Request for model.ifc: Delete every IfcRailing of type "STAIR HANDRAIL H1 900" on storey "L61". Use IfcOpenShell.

First a look at what the model holds.

```python
import ifcopenshell
import ifcopenshell.util.element

model = ifcopenshell.open("model.ifc")
print(model.schema)
storey = next(s for s in model.by_type("IfcBuildingStorey") if s.Name == "L61")
railings = [e for e in ifcopenshell.util.element.get_decomposition(storey) if e.is_a("IfcRailing")]
seen = {}
for e in railings:
    element_type = ifcopenshell.util.element.get_type(e)
    name = element_type.Name if element_type not in (None, e) else None
    seen[name] = seen.get(name, 0) + 1
for name, count in sorted(seen.items(), key=str):
    print(count, "x", name)
```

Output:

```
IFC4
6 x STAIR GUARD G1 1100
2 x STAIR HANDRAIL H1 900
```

```python
import ifcopenshell
import ifcopenshell.api.root
import ifcopenshell.util.element

model = ifcopenshell.open("model.ifc")

storey = next(s for s in model.by_type("IfcBuildingStorey") if s.Name == "L61")
railings = [e for e in ifcopenshell.util.element.get_decomposition(storey) if e.is_a("IfcRailing")]
targets = [e for e in railings if (t := ifcopenshell.util.element.get_type(e)) not in (None, e) and t.Name == "STAIR HANDRAIL H1 900"]

for e in targets:
    ifcopenshell.api.root.remove_product(model, product=e)
print(len(targets), "removed")

model.write("model_v2.ifc")
```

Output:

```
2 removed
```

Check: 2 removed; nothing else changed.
